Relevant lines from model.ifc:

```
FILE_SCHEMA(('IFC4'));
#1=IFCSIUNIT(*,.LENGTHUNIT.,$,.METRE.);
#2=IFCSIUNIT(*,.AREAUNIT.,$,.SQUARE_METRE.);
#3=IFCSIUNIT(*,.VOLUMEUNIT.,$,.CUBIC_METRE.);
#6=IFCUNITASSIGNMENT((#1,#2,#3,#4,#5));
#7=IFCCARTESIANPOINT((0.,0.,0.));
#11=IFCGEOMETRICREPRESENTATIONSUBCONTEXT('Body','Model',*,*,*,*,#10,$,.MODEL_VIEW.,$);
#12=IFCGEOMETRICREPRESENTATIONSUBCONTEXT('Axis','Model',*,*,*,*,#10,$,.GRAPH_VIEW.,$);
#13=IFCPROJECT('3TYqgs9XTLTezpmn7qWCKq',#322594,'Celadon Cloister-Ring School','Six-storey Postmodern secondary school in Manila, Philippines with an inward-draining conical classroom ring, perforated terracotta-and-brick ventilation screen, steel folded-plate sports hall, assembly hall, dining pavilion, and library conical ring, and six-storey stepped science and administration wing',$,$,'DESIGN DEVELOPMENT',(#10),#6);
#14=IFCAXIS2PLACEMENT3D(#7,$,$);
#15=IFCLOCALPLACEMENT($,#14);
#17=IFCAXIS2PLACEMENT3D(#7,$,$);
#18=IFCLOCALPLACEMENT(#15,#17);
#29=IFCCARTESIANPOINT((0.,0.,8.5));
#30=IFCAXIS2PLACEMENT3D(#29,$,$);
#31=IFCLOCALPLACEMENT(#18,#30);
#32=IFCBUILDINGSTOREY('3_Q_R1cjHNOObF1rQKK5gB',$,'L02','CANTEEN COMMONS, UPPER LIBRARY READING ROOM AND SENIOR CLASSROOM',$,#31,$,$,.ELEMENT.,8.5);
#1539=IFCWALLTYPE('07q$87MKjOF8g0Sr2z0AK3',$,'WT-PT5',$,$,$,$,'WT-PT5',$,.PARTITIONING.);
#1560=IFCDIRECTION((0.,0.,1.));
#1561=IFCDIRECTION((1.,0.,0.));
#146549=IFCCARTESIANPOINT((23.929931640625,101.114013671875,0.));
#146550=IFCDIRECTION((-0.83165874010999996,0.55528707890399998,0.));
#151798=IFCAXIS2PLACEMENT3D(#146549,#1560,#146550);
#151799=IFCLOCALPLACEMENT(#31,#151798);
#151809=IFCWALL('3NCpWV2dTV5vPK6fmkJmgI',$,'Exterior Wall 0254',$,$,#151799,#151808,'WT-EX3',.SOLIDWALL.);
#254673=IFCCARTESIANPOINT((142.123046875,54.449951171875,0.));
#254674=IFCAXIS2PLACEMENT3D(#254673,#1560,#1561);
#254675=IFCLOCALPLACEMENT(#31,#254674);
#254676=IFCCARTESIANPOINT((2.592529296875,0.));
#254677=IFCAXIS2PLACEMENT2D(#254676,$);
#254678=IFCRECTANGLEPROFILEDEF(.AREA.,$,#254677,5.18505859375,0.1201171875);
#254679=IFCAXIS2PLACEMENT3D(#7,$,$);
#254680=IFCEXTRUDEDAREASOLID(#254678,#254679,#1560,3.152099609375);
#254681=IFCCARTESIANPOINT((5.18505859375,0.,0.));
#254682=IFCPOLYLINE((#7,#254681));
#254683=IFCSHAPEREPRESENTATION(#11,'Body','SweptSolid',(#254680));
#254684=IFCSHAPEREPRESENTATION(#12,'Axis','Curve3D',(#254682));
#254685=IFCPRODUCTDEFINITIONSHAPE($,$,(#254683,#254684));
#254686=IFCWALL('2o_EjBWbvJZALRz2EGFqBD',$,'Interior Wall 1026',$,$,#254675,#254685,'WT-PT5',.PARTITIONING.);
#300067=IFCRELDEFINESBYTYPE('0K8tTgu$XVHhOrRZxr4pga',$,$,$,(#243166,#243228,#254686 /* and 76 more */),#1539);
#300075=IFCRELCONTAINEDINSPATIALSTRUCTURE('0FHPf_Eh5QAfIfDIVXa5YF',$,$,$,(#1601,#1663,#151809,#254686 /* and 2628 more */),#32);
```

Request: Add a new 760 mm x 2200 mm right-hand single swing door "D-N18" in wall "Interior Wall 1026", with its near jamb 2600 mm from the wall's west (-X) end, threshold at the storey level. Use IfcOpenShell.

```python
import numpy as np
import ifcopenshell
import ifcopenshell.api.feature
import ifcopenshell.api.geometry
import ifcopenshell.api.root
import ifcopenshell.api.spatial
import ifcopenshell.geom
import ifcopenshell.util.element
import ifcopenshell.util.placement
import ifcopenshell.util.representation
import ifcopenshell.util.shape
import ifcopenshell.util.unit

model = ifcopenshell.open("model.ifc")
unit_scale = ifcopenshell.util.unit.calculate_unit_scale(model)
settings = ifcopenshell.geom.settings()


def volume(element):
    """Net volume in cubic metres, openings subtracted."""
    shape = ifcopenshell.geom.create_shape(settings, element)
    return ifcopenshell.util.shape.get_volume(shape.geometry)


wall = model.by_id(254686)
storey = ifcopenshell.util.element.get_container(wall, ifc_class="IfcBuildingStorey")
context = ifcopenshell.util.representation.get_context(model, "Model", "Body", "MODEL_VIEW")
before = volume(wall)

width, height, from_end, sill = 0.76, 2.2, 2.6, 0.0  # metres

# The wall runs along its own X axis, and the end named is its -X end.
wall_shape = ifcopenshell.geom.create_shape(settings, wall)
x, y, z = ifcopenshell.util.shape.get_vertices(wall_shape.geometry).T
start = x.min() + from_end
face, thickness = float(y.min()), float(y.max() - y.min())
wall_matrix = ifcopenshell.util.placement.get_local_placement(wall.ObjectPlacement)
level = ifcopenshell.util.placement.get_local_placement(storey.ObjectPlacement)[2, 3]


def in_wall(x, y):
    """Placement at x, y metres in the wall's axes, at sill height."""
    matrix = wall_matrix.copy()
    matrix[:, 3] = wall_matrix @ np.array([x / unit_scale, y / unit_scale, 0.0, 1.0])
    matrix[2, 3] = level + sill / unit_scale
    return matrix


# Opening: a box that overshoots both wall faces by 50 mm.
opening = ifcopenshell.api.root.create_entity(model, ifc_class="IfcOpeningElement", predefined_type="OPENING")
box = ifcopenshell.api.geometry.add_wall_representation(
    model, context=context, length=width, height=height, thickness=thickness + 0.1
)
ifcopenshell.api.geometry.assign_representation(model, product=opening, representation=box)
ifcopenshell.api.geometry.edit_object_placement(model, product=opening, matrix=in_wall(start, face - 0.05), is_si=False)
ifcopenshell.api.feature.add_feature(model, feature=opening, element=wall)

door = ifcopenshell.api.root.create_entity(model, ifc_class="IfcDoor", name="D-N18", predefined_type="DOOR")
door.OverallWidth, door.OverallHeight = width / unit_scale, height / unit_scale
door.OperationType = "SINGLE_SWING_RIGHT"
body = ifcopenshell.api.geometry.add_door_representation(
    model,
    context=context,
    overall_width=door.OverallWidth,
    overall_height=door.OverallHeight,
    operation_type="SINGLE_SWING_RIGHT",
    lining_properties={"LiningDepth": thickness / unit_scale, "ThresholdDepth": thickness / unit_scale},
)
ifcopenshell.api.geometry.assign_representation(model, product=door, representation=body)
ifcopenshell.api.spatial.assign_container(model, products=[door], relating_structure=storey)
ifcopenshell.api.feature.add_filling(model, opening=opening, element=door)

# The lining spans the wall, so the door starts at the wall face.
ifcopenshell.api.geometry.edit_object_placement(model, product=door, matrix=in_wall(start, face), is_si=False)

after = volume(wall)

print(f"wall volume {before:.3f} -> {after:.3f} m3")

model.write("model_edited.ifc")
```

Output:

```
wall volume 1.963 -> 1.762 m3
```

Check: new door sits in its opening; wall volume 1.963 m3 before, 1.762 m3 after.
